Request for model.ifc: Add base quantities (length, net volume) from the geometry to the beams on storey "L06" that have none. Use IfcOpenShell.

First a look at what the model holds.

```python
import ifcopenshell
import ifcopenshell.util.element
import ifcopenshell.util.unit

model = ifcopenshell.open("model.ifc")
print(model.schema)
for unit_type in ("LENGTHUNIT", "AREAUNIT", "VOLUMEUNIT"):
    print(unit_type, ifcopenshell.util.unit.calculate_unit_scale(model, unit_type))
storey = next(s for s in model.by_type("IfcBuildingStorey") if s.Name == "L06")
beams = [e for e in ifcopenshell.util.element.get_decomposition(storey) if e.is_a("IfcBeam")]
for e in sorted(beams, key=lambda e: e.id()):
    print(e.id(), e.is_a(), e.Name, list(ifcopenshell.util.element.get_psets(e, qtos_only=True)), sep=" | ")
```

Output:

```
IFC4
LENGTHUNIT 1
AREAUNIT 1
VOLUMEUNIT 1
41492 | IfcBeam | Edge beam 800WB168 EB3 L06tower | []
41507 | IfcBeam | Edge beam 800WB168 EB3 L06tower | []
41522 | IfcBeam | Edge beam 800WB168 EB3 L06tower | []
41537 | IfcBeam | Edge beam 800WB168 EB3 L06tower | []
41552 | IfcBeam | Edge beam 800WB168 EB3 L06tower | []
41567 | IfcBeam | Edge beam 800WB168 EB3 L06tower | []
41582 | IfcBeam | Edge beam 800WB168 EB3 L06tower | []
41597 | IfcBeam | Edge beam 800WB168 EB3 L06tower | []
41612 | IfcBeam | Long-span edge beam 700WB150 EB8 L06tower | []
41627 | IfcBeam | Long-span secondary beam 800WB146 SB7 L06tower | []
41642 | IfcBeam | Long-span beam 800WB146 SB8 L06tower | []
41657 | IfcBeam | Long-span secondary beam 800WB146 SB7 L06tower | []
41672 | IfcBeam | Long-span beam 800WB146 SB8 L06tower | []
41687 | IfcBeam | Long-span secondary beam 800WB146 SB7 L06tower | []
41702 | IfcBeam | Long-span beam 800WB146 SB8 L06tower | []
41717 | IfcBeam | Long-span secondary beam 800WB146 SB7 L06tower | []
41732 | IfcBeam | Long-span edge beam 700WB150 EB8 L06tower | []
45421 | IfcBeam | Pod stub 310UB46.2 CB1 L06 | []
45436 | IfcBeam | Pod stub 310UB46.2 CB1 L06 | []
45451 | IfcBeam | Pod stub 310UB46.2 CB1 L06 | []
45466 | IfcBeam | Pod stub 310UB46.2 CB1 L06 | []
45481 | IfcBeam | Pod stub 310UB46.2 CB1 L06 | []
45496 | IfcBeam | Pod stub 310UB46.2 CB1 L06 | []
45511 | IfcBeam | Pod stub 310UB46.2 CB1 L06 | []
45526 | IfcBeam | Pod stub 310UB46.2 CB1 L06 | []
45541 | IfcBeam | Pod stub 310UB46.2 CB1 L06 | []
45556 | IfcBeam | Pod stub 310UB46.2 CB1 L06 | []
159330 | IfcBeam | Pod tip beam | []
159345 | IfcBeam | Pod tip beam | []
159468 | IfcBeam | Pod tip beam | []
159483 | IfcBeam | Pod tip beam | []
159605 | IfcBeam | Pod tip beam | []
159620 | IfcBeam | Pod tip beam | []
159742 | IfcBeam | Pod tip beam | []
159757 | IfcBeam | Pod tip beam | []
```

```python
import ifcopenshell
import ifcopenshell.api.pset
import ifcopenshell.geom
import ifcopenshell.util.element
import ifcopenshell.util.shape
import ifcopenshell.util.unit

model = ifcopenshell.open("model.ifc")
unit_scale = ifcopenshell.util.unit.calculate_unit_scale(model)
volume_scale = ifcopenshell.util.unit.calculate_unit_scale(model, "VOLUMEUNIT")
settings = ifcopenshell.geom.settings()

storey = next(s for s in model.by_type("IfcBuildingStorey") if s.Name == "L06")
beams = [e for e in ifcopenshell.util.element.get_decomposition(storey) if e.is_a("IfcBeam")]

for e in sorted(beams, key=lambda e: e.id()):
    if ifcopenshell.util.element.get_psets(e, qtos_only=True, should_inherit=False):
        continue
    # Geometry comes back in metres, in the element's own axes.
    shape = ifcopenshell.geom.create_shape(settings, e)
    values = {
        "Length": ifcopenshell.util.shape.get_max_xyz(shape.geometry) / unit_scale,
        "NetVolume": ifcopenshell.util.shape.get_volume(shape.geometry) / volume_scale,
    }
    qto = ifcopenshell.api.pset.add_qto(model, product=e, name="Qto_BeamBaseQuantities")
    ifcopenshell.api.pset.edit_qto(model, qto=qto, properties=values)
    print(e.id(), {k: round(v, 3) for k, v in values.items()})

model.write("model_v2.ifc")
```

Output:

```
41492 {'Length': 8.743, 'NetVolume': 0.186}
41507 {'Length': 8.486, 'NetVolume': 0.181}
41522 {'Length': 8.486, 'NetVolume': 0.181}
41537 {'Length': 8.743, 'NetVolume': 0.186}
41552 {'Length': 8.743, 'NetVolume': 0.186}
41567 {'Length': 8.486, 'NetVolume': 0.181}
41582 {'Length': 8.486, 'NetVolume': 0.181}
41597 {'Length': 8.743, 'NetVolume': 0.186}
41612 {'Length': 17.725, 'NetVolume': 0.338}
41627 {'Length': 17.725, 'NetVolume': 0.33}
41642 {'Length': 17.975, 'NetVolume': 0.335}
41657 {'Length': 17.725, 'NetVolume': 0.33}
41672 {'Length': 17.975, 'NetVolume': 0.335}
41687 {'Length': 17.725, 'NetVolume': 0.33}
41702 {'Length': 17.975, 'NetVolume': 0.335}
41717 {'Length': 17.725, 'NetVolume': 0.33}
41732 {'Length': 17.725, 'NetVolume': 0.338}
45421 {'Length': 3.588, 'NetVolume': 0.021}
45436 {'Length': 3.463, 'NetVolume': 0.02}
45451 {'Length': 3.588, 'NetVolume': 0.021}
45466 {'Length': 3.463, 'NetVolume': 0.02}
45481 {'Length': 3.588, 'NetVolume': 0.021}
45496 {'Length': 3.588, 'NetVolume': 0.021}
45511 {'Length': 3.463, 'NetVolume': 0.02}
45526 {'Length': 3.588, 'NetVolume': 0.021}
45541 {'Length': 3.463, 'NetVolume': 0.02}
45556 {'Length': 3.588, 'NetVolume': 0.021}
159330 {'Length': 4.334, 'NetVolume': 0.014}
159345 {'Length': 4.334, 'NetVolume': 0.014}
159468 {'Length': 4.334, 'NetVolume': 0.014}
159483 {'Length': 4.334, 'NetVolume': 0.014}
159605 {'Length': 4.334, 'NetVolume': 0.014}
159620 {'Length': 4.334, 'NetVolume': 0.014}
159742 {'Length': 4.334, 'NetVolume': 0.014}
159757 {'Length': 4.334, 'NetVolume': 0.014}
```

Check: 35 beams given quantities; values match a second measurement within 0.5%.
